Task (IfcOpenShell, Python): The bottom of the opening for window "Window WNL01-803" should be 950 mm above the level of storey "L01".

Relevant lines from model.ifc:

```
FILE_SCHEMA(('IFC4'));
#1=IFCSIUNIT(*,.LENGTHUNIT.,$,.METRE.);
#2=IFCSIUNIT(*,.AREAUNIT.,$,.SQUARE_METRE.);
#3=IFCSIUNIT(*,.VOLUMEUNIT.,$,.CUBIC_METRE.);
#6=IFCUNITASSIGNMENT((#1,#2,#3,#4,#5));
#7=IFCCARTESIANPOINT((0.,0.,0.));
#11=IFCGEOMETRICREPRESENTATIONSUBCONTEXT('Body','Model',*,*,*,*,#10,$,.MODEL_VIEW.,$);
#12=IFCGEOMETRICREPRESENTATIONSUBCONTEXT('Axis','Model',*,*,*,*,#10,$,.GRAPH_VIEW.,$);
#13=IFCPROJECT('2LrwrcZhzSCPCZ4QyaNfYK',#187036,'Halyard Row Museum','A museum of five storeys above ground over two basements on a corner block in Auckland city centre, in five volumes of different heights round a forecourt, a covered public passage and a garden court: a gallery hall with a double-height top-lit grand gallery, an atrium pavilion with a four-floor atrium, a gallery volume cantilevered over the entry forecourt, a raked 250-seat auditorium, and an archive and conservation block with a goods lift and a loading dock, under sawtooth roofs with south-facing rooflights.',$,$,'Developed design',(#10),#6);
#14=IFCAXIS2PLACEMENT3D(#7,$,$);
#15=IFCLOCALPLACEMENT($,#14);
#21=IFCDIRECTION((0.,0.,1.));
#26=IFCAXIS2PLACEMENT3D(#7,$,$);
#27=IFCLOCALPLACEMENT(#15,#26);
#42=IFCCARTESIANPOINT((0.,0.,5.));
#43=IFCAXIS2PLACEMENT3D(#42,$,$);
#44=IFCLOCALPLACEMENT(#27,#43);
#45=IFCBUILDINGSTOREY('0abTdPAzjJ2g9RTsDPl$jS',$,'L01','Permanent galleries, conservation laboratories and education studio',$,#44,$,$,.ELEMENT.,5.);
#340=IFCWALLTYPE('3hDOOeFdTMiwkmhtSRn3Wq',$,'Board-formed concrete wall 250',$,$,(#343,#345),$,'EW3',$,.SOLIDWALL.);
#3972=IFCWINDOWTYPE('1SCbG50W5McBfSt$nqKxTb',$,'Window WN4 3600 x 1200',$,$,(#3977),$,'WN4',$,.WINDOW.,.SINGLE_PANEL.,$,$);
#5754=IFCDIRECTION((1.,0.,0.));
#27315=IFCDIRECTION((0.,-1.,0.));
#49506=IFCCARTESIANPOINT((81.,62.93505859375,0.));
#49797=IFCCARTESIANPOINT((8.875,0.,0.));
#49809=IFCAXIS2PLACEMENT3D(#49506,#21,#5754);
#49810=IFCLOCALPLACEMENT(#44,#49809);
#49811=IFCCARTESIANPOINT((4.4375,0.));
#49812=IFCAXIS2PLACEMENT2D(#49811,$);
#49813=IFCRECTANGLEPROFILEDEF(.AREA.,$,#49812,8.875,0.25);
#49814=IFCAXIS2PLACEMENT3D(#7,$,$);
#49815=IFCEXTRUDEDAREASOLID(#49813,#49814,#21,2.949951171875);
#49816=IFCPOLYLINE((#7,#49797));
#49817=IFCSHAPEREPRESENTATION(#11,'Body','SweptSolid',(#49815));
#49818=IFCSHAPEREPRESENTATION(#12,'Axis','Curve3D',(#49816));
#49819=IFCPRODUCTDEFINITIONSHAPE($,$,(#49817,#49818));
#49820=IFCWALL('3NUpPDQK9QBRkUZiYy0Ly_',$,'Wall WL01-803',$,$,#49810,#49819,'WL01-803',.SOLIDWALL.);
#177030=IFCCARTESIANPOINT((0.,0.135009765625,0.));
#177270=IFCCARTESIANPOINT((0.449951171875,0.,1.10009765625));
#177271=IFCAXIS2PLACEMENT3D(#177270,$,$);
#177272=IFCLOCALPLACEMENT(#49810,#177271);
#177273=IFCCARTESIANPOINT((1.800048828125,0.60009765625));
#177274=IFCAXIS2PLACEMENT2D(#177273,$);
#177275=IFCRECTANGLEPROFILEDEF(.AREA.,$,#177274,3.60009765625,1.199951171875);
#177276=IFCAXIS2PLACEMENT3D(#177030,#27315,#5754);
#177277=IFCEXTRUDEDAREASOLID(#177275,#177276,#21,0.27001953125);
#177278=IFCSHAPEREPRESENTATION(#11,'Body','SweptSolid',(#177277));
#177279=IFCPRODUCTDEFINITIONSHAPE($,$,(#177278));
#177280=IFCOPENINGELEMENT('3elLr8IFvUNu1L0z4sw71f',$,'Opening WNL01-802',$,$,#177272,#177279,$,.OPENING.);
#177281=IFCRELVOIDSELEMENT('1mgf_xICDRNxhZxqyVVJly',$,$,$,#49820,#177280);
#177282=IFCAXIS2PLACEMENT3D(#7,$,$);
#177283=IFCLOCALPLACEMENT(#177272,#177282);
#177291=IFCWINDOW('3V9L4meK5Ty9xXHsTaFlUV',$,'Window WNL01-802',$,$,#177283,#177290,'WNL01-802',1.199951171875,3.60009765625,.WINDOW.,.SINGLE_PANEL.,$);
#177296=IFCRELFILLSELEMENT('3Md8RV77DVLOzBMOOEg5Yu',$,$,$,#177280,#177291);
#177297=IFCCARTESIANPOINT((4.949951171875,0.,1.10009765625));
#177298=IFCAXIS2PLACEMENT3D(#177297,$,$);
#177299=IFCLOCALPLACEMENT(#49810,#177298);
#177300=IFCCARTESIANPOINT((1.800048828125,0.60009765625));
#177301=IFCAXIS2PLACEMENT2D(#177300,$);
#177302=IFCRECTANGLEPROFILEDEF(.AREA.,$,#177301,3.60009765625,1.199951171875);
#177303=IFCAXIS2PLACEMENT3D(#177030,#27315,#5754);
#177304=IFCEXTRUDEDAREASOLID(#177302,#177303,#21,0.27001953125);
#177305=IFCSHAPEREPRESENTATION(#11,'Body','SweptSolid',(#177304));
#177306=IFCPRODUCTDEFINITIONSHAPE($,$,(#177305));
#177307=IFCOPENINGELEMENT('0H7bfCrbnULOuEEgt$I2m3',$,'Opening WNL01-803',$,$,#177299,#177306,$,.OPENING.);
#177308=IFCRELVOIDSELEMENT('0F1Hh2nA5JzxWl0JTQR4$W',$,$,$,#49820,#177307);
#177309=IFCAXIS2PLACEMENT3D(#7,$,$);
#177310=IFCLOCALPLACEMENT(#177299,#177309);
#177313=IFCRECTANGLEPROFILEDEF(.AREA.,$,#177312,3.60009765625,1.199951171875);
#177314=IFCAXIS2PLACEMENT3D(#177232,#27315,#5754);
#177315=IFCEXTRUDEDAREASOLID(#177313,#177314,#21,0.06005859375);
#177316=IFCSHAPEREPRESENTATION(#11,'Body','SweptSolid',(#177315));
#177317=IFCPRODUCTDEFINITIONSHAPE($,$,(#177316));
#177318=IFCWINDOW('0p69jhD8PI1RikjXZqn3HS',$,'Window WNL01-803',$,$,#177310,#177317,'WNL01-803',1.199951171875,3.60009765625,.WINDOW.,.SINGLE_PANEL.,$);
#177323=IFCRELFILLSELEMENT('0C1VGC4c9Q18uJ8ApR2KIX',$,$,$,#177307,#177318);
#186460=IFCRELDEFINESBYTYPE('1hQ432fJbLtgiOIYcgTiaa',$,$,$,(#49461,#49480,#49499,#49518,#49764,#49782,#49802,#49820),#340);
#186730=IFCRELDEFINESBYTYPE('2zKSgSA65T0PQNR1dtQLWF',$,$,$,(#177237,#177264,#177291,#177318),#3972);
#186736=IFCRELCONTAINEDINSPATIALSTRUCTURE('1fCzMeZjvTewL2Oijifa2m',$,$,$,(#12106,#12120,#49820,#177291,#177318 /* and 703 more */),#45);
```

```python
import numpy as np
import ifcopenshell
import ifcopenshell.api.geometry
import ifcopenshell.geom
import ifcopenshell.util.element
import ifcopenshell.util.placement
import ifcopenshell.util.shape
import ifcopenshell.util.unit

model = ifcopenshell.open("model.ifc")
unit_scale = ifcopenshell.util.unit.calculate_unit_scale(model)

window = model.by_guid("0p69jhD8PI1RikjXZqn3HS")
opening = window.FillsVoids[0].RelatingOpeningElement
storey = ifcopenshell.util.element.get_container(window, ifc_class="IfcBuildingStorey")
level = ifcopenshell.util.placement.get_local_placement(storey.ObjectPlacement)[2, 3]

# The opening's origin need not be at the sill, so measure its lowest point.
shape = ifcopenshell.geom.create_shape(ifcopenshell.geom.settings(), opening)
bottom = ifcopenshell.util.shape.get_shape_bottom_elevation(shape, shape.geometry) / unit_scale
dz = level + 0.95 - bottom

shift = np.array([0.0, 0.0, dz])
# The window is placed relative to its opening, so it follows when the opening moves.
matrix = ifcopenshell.util.placement.get_local_placement(opening.ObjectPlacement)
matrix[:3, 3] += shift
ifcopenshell.api.geometry.edit_object_placement(
    model, product=opening, matrix=matrix, is_si=False, should_transform_children=True
)

print(f"moved by {dz * unit_scale:+.3f} m")

model.write("model_edited.ifc")
```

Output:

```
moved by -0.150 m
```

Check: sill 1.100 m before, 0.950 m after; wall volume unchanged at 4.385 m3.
